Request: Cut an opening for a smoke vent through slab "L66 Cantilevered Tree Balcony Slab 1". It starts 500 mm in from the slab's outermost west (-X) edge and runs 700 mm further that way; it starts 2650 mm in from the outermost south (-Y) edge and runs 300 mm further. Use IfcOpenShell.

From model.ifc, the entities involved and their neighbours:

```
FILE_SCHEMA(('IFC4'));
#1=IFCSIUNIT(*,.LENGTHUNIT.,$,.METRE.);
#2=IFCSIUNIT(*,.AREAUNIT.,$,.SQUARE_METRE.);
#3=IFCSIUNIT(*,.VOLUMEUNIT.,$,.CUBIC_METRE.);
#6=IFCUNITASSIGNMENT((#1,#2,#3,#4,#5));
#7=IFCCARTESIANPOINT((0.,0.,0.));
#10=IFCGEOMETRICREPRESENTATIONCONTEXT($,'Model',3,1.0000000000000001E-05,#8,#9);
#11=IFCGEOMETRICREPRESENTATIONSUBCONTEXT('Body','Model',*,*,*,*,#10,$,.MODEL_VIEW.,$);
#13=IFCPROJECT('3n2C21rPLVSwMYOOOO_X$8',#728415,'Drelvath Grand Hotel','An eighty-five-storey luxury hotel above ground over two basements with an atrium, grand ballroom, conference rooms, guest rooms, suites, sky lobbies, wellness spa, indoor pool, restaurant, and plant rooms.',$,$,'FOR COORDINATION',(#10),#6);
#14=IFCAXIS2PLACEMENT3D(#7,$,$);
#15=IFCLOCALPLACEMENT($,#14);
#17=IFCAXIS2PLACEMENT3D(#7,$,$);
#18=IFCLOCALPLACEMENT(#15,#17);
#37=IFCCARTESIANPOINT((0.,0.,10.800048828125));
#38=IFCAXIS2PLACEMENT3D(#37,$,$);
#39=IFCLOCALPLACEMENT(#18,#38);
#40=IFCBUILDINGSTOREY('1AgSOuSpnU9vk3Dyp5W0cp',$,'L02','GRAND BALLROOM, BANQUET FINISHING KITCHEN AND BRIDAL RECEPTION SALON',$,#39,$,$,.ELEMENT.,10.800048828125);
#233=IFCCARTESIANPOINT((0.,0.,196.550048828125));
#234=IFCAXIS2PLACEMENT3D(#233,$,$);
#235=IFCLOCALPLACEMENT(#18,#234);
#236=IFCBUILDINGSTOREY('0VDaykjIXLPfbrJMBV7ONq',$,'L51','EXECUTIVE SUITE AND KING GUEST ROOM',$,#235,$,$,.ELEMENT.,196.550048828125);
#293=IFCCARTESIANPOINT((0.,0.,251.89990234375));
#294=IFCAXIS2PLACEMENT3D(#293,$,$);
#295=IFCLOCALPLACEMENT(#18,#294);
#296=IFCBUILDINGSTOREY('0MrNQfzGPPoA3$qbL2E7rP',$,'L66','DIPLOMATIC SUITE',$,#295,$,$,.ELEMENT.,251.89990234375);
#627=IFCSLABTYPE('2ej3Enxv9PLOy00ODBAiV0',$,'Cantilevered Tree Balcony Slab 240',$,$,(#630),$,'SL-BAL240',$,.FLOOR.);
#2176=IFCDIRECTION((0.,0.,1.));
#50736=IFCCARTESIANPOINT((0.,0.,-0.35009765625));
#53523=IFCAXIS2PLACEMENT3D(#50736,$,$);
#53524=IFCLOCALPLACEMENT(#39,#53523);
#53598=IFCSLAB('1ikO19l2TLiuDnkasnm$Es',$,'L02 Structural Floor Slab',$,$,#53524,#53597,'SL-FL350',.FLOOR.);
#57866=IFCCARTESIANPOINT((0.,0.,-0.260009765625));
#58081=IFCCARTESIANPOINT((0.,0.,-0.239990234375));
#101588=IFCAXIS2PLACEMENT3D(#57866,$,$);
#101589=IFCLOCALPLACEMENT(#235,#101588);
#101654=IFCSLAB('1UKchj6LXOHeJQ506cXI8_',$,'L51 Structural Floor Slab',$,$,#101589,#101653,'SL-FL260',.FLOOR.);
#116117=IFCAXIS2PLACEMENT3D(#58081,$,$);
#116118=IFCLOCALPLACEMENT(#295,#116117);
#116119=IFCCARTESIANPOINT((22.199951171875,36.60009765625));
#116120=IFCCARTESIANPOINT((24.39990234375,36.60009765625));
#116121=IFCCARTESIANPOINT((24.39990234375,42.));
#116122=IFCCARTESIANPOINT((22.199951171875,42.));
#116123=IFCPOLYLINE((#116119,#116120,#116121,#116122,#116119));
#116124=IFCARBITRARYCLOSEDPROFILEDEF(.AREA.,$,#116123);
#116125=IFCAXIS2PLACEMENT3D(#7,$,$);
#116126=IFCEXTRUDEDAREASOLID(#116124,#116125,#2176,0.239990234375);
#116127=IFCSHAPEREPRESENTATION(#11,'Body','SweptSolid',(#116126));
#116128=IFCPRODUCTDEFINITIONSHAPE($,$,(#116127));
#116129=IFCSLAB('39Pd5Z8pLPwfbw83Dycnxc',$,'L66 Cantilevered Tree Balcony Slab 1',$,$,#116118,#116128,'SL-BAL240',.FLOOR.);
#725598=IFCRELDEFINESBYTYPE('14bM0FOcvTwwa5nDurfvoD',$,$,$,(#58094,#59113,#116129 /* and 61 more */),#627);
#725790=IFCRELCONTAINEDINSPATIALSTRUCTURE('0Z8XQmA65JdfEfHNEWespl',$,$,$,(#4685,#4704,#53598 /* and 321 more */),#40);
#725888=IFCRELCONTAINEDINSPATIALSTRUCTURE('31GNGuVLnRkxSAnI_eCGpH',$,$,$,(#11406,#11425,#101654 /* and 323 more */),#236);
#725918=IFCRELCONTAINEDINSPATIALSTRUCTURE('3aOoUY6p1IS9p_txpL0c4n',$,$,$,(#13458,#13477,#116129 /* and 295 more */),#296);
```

```python
import numpy as np
import ifcopenshell
import ifcopenshell.api.feature
import ifcopenshell.api.geometry
import ifcopenshell.api.root
import ifcopenshell.geom
import ifcopenshell.util.placement
import ifcopenshell.util.representation
import ifcopenshell.util.shape
import ifcopenshell.util.unit

model = ifcopenshell.open("model.ifc")
unit_scale = ifcopenshell.util.unit.calculate_unit_scale(model)
settings = ifcopenshell.geom.settings()


def volume(element):
    """Net volume in cubic metres, openings subtracted."""
    shape = ifcopenshell.geom.create_shape(settings, element)
    return ifcopenshell.util.shape.get_volume(shape.geometry)


slab = model.by_guid("39Pd5Z8pLPwfbw83Dycnxc")
before = volume(slab)

# Extent in the slab's own axes, in metres. The edges named are its -X and -Y sides.
slab_shape = ifcopenshell.geom.create_shape(settings, slab)
vertices = ifcopenshell.util.shape.get_vertices(slab_shape.geometry)
x_min, y_min, bottom = vertices.min(axis=0)
top = vertices[:, 2].max()

opening = ifcopenshell.api.root.create_entity(model, ifc_class="IfcOpeningElement", name="Smoke vent opening", predefined_type="OPENING")
context = ifcopenshell.util.representation.get_context(model, "Model", "Body", "MODEL_VIEW")
width, depth = 0.7, 0.3
outline = [(0.0, 0.0), (width, 0.0), (width, depth), (0.0, depth), (0.0, 0.0)]
# Overshoot both faces by 50 mm so the cut is clean.
shape = ifcopenshell.api.geometry.add_slab_representation(
    model, context=context, depth=top - bottom + 0.1, polyline=outline
)
ifcopenshell.api.geometry.assign_representation(model, product=opening, representation=shape)

matrix = ifcopenshell.util.placement.get_local_placement(slab.ObjectPlacement)
matrix[:, 3] = matrix @ np.append(np.array([x_min + 0.5, y_min + 2.65, bottom - 0.05]) / unit_scale, 1.0)
ifcopenshell.api.geometry.edit_object_placement(model, product=opening, matrix=matrix, is_si=False)
ifcopenshell.api.feature.add_feature(model, feature=opening, element=slab)

after = volume(slab)

print(f"slab volume {before:.3f} -> {after:.3f} m3")

model.write("model_v2.ifc")
```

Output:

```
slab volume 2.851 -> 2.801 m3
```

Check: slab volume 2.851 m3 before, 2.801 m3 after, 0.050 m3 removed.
